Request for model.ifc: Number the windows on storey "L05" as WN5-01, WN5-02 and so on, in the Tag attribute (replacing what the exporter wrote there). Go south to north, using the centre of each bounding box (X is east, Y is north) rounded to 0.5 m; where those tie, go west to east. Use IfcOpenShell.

First a look at what the model holds.

```python
import ifcopenshell
import ifcopenshell.util.element
import ifcopenshell.util.placement

model = ifcopenshell.open("model.ifc")
print(model.schema)
storey = next(s for s in model.by_type("IfcBuildingStorey") if s.Name == "L05")
windows = [e for e in ifcopenshell.util.element.get_decomposition(storey) if e.is_a("IfcWindow")]
for e in sorted(windows, key=lambda e: e.id()):
    origin = ifcopenshell.util.placement.get_local_placement(e.ObjectPlacement)[:3, 3]
    print(e.id(), e.Tag, e.Name, origin.round(2) + 0.0, sep=" | ")
```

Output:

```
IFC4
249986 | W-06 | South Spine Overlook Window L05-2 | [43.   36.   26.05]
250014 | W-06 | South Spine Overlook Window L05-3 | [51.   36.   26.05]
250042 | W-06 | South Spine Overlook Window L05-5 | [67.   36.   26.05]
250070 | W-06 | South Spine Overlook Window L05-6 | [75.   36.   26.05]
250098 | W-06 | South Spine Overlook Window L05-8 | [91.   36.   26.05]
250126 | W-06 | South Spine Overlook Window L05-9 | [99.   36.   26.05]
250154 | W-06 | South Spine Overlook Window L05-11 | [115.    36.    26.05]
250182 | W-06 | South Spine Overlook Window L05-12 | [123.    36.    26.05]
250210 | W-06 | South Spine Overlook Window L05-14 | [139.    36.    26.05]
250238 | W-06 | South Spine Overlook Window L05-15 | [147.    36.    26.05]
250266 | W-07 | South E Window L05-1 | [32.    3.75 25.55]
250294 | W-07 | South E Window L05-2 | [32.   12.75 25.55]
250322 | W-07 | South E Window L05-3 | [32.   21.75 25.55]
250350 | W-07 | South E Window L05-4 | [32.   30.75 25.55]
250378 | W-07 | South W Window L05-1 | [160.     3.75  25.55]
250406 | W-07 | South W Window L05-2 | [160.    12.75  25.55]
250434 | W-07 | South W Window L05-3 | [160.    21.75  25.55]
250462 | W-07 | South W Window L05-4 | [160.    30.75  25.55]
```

```python
import ifcopenshell
import ifcopenshell.geom
import ifcopenshell.util.element
import ifcopenshell.util.shape

model = ifcopenshell.open("model.ifc")
settings = ifcopenshell.geom.settings()
settings.set("use-world-coords", True)


def centre(element):
    shape = ifcopenshell.geom.create_shape(settings, element)
    return ifcopenshell.util.shape.get_bbox_centroid(shape.geometry)


storey = next(s for s in model.by_type("IfcBuildingStorey") if s.Name == "L05")
windows = [e for e in ifcopenshell.util.element.get_decomposition(storey) if e.is_a("IfcWindow")]

# Insertion points can sit at a corner or the storey origin, so sort by the geometry (in metres).
centres = {e: centre(e) for e in windows}
windows.sort(key=lambda e: (round(centres[e][1] / 0.5), centres[e][0]))

for i, e in enumerate(windows, start=1):
    number = f"WN5-{i:02d}"
    e.Tag = number
    print(e.id(), number)

model.write("model_edited.ifc")
```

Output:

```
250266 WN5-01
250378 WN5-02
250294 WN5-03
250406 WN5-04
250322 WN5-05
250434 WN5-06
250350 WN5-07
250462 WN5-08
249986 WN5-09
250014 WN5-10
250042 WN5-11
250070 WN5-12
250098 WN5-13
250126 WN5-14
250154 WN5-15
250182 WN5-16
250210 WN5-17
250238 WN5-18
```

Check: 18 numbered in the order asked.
